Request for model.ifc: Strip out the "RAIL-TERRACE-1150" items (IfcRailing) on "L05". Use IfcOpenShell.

First a look at what the model holds.

```python
import ifcopenshell
import ifcopenshell.util.element

model = ifcopenshell.open("model.ifc")
print(model.schema)
storey = next(s for s in model.by_type("IfcBuildingStorey") if s.Name == "L05")
railings = [e for e in ifcopenshell.util.element.get_decomposition(storey) if e.is_a("IfcRailing")]
seen = {}
for e in railings:
    element_type = ifcopenshell.util.element.get_type(e)
    name = element_type.Name if element_type not in (None, e) else None
    seen[name] = seen.get(name, 0) + 1
for name, count in sorted(seen.items(), key=str):
    print(count, "x", name)
```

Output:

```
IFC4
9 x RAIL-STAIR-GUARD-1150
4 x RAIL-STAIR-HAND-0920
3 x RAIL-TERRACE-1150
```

```python
import ifcopenshell
import ifcopenshell.api.root
import ifcopenshell.util.element

model = ifcopenshell.open("model.ifc")

storey = next(s for s in model.by_type("IfcBuildingStorey") if s.Name == "L05")
railings = [e for e in ifcopenshell.util.element.get_decomposition(storey) if e.is_a("IfcRailing")]
targets = [e for e in railings if (t := ifcopenshell.util.element.get_type(e)) not in (None, e) and t.Name == "RAIL-TERRACE-1150"]

for e in targets:
    ifcopenshell.api.root.remove_product(model, product=e)
print(len(targets), "removed")

model.write("model_updated.ifc")
```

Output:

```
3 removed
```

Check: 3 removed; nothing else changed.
